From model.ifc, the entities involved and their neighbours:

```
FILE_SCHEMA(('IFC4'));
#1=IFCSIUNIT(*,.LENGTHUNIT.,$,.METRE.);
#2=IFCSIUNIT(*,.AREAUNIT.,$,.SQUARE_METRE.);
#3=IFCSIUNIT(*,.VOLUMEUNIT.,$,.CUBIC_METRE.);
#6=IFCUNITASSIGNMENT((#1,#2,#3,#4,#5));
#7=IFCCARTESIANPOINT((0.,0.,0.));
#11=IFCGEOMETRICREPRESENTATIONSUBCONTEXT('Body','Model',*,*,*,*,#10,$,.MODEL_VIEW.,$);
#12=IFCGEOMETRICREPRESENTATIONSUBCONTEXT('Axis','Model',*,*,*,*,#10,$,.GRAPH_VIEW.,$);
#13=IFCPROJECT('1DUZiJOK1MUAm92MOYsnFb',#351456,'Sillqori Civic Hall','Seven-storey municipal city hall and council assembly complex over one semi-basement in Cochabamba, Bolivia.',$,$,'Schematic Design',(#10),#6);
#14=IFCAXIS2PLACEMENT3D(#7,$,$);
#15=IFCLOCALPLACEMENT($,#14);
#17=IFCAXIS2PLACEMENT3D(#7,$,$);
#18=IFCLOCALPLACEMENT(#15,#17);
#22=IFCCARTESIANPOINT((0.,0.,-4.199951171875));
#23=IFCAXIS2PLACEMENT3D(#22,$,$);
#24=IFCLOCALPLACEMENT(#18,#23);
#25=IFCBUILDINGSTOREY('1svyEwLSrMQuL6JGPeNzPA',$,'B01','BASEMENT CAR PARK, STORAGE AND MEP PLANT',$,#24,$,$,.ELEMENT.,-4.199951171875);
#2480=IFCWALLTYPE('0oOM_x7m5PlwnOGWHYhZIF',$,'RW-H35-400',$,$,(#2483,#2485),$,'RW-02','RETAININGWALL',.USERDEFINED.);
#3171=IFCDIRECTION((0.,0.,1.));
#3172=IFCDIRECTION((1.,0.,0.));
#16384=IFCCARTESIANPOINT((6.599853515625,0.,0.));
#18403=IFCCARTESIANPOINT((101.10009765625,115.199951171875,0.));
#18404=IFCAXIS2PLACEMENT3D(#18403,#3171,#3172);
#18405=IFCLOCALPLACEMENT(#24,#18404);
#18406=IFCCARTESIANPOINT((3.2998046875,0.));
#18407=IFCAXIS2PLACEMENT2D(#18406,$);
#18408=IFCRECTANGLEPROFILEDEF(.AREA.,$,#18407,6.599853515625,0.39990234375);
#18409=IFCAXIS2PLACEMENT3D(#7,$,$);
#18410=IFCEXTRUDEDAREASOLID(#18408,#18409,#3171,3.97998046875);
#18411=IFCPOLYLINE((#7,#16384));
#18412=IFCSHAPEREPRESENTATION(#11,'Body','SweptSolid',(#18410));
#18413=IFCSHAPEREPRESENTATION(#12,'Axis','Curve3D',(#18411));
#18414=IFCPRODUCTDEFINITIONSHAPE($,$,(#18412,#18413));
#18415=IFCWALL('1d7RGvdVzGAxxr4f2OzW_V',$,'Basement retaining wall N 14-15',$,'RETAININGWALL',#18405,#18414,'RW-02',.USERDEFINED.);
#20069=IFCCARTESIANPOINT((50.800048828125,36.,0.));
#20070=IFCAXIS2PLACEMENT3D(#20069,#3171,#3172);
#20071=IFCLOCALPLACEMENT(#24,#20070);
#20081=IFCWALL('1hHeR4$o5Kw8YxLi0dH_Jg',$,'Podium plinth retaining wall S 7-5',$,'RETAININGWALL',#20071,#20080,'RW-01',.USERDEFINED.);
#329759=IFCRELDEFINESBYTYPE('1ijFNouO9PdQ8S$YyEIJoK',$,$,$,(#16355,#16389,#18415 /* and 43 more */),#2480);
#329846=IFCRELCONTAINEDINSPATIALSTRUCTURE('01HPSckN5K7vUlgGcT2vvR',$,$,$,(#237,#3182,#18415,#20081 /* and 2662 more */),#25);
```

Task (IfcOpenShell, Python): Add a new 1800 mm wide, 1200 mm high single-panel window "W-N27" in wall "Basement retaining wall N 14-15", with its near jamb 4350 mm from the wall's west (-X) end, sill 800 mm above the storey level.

```python
import numpy as np
import ifcopenshell
import ifcopenshell.api.feature
import ifcopenshell.api.geometry
import ifcopenshell.api.root
import ifcopenshell.api.spatial
import ifcopenshell.geom
import ifcopenshell.util.element
import ifcopenshell.util.placement
import ifcopenshell.util.representation
import ifcopenshell.util.shape
import ifcopenshell.util.unit

model = ifcopenshell.open("model.ifc")
unit_scale = ifcopenshell.util.unit.calculate_unit_scale(model)
settings = ifcopenshell.geom.settings()


def volume(element):
    """Net volume in cubic metres, openings subtracted."""
    shape = ifcopenshell.geom.create_shape(settings, element)
    return ifcopenshell.util.shape.get_volume(shape.geometry)


wall = model.by_guid("1d7RGvdVzGAxxr4f2OzW_V")
storey = ifcopenshell.util.element.get_container(wall, ifc_class="IfcBuildingStorey")
context = ifcopenshell.util.representation.get_context(model, "Model", "Body", "MODEL_VIEW")
before = volume(wall)

width, height, from_end, sill = 1.8, 1.2, 4.35, 0.8  # metres

# The wall runs along its own X axis, and the end named is its -X end.
wall_shape = ifcopenshell.geom.create_shape(settings, wall)
x, y, z = ifcopenshell.util.shape.get_vertices(wall_shape.geometry).T
start = x.min() + from_end
face, thickness = float(y.min()), float(y.max() - y.min())
wall_matrix = ifcopenshell.util.placement.get_local_placement(wall.ObjectPlacement)
level = ifcopenshell.util.placement.get_local_placement(storey.ObjectPlacement)[2, 3]


def in_wall(x, y):
    """Placement at x, y metres in the wall's axes, at sill height."""
    matrix = wall_matrix.copy()
    matrix[:, 3] = wall_matrix @ np.array([x / unit_scale, y / unit_scale, 0.0, 1.0])
    matrix[2, 3] = level + sill / unit_scale
    return matrix


# Opening: a box that overshoots both wall faces by 50 mm.
opening = ifcopenshell.api.root.create_entity(model, ifc_class="IfcOpeningElement", predefined_type="OPENING")
box = ifcopenshell.api.geometry.add_wall_representation(
    model, context=context, length=width, height=height, thickness=thickness + 0.1
)
ifcopenshell.api.geometry.assign_representation(model, product=opening, representation=box)
ifcopenshell.api.geometry.edit_object_placement(model, product=opening, matrix=in_wall(start, face - 0.05), is_si=False)
ifcopenshell.api.feature.add_feature(model, feature=opening, element=wall)

window = ifcopenshell.api.root.create_entity(model, ifc_class="IfcWindow", name="W-N27", predefined_type="WINDOW")
window.OverallWidth, window.OverallHeight = width / unit_scale, height / unit_scale
window.PartitioningType = "SINGLE_PANEL"
body = ifcopenshell.api.geometry.add_window_representation(
    model,
    context=context,
    overall_width=window.OverallWidth,
    overall_height=window.OverallHeight,
    partition_type="SINGLE_PANEL",
)
ifcopenshell.api.geometry.assign_representation(model, product=window, representation=body)
ifcopenshell.api.spatial.assign_container(model, products=[window], relating_structure=storey)
ifcopenshell.api.feature.add_filling(model, opening=opening, element=window)

# Centre the window in the wall's thickness.
ifcopenshell.api.geometry.edit_object_placement(model, product=window, matrix=in_wall(start, face), is_si=False)
window_shape = ifcopenshell.geom.create_shape(settings, window)
depth = ifcopenshell.util.shape.get_vertices(window_shape.geometry)[:, 1]
offset = face + thickness / 2 - (depth.min() + depth.max()) / 2
ifcopenshell.api.geometry.edit_object_placement(model, product=window, matrix=in_wall(start, offset), is_si=False)

after = volume(wall)

print(f"wall volume {before:.3f} -> {after:.3f} m3")

model.write("model-out.ifc")
```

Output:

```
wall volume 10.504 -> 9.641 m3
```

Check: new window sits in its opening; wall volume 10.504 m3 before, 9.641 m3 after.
